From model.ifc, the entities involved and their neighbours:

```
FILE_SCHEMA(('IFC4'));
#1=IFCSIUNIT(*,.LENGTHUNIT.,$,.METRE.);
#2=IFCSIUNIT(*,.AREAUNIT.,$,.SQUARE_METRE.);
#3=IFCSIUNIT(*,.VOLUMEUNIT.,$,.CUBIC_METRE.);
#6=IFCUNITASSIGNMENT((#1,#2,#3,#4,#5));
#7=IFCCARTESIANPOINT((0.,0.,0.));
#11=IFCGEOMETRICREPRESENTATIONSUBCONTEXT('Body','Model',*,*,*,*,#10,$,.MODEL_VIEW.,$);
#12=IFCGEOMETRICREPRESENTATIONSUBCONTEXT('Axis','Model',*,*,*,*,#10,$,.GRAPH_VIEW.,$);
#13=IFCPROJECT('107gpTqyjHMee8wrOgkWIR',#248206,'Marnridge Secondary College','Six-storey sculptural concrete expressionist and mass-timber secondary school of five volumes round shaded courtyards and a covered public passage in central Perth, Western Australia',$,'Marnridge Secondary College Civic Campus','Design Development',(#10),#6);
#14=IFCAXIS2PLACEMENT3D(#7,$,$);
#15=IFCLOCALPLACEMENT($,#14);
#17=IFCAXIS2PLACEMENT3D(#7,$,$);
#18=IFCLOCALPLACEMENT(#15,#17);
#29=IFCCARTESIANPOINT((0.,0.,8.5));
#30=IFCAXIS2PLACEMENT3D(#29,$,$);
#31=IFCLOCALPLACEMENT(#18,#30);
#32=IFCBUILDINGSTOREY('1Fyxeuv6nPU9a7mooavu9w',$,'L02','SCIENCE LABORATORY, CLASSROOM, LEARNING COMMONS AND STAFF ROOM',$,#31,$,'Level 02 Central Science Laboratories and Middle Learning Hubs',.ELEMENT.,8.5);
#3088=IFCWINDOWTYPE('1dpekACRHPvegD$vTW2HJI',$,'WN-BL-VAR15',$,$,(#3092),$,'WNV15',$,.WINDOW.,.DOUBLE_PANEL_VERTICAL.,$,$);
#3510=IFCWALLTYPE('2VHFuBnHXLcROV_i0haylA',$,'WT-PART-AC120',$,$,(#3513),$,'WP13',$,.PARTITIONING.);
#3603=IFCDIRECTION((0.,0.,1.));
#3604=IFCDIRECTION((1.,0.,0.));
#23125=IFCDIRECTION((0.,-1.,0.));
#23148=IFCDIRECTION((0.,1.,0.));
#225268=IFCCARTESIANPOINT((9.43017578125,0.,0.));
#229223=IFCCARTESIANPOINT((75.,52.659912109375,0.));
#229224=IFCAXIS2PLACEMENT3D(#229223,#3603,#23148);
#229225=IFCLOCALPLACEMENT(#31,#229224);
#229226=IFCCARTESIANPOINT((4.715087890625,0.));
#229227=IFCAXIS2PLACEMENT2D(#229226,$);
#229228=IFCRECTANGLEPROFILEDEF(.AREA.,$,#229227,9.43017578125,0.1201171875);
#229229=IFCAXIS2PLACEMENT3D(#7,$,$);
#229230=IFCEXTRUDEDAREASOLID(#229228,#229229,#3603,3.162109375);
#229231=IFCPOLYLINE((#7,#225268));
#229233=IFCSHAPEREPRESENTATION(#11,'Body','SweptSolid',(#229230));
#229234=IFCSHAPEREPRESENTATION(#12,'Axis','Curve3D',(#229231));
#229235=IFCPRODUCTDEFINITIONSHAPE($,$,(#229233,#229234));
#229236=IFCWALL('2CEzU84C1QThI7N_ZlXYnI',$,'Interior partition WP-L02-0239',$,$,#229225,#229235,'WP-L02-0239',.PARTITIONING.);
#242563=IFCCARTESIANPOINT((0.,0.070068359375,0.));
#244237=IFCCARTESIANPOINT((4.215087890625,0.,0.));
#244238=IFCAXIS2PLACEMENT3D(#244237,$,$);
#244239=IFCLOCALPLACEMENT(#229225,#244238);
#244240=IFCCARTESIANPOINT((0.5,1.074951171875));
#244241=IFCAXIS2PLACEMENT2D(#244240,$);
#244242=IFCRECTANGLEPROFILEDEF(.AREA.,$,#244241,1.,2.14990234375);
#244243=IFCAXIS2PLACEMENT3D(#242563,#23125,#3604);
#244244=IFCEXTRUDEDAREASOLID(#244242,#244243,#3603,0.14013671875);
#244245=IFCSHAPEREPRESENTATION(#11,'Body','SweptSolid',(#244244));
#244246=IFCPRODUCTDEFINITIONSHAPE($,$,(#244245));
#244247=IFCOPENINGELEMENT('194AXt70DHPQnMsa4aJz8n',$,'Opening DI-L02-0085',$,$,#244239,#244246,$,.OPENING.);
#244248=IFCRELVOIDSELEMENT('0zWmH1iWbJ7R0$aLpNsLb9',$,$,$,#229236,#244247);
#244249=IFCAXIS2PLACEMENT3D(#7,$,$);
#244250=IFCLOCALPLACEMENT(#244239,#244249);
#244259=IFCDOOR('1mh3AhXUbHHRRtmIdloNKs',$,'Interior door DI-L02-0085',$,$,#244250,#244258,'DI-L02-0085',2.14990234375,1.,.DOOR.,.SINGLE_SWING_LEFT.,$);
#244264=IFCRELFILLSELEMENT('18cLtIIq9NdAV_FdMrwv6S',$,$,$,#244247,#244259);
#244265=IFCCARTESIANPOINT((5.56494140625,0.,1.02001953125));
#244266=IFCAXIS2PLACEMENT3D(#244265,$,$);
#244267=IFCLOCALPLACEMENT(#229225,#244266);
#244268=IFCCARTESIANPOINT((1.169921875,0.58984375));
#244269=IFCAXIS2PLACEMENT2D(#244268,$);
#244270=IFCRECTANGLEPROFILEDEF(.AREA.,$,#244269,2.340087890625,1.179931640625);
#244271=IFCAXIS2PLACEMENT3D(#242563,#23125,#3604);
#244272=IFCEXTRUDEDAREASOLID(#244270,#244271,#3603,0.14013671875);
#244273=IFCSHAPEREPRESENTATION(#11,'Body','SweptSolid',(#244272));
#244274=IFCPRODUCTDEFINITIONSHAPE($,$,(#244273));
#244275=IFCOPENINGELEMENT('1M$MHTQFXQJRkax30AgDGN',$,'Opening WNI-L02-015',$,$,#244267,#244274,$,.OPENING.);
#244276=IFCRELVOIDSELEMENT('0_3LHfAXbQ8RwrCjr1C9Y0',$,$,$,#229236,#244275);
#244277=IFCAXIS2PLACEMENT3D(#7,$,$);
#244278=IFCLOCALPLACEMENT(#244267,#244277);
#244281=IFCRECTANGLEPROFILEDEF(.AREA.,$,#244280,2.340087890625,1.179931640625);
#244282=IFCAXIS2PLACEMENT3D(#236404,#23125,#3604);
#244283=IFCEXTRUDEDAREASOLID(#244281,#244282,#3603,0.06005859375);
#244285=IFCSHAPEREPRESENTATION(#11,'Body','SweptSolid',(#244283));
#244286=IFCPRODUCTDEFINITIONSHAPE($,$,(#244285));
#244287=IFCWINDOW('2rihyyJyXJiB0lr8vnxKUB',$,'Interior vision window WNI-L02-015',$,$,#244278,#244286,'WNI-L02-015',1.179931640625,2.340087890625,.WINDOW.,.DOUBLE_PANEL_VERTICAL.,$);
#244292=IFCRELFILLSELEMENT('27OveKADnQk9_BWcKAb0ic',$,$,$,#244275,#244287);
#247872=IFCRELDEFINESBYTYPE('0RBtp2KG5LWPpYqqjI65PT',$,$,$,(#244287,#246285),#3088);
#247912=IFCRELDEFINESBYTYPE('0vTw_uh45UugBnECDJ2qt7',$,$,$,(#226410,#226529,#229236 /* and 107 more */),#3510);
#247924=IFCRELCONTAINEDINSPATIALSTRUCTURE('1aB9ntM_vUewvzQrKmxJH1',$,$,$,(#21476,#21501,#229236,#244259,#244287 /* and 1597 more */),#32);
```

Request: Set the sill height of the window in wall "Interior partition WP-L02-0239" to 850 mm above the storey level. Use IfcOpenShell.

```python
import numpy as np
import ifcopenshell
import ifcopenshell.api.geometry
import ifcopenshell.geom
import ifcopenshell.util.element
import ifcopenshell.util.placement
import ifcopenshell.util.shape
import ifcopenshell.util.unit

model = ifcopenshell.open("model.ifc")
unit_scale = ifcopenshell.util.unit.calculate_unit_scale(model)

window = model.by_guid("2rihyyJyXJiB0lr8vnxKUB")
opening = window.FillsVoids[0].RelatingOpeningElement
storey = ifcopenshell.util.element.get_container(window, ifc_class="IfcBuildingStorey")
level = ifcopenshell.util.placement.get_local_placement(storey.ObjectPlacement)[2, 3]

# The opening's origin need not be at the sill, so measure its lowest point.
shape = ifcopenshell.geom.create_shape(ifcopenshell.geom.settings(), opening)
bottom = ifcopenshell.util.shape.get_shape_bottom_elevation(shape, shape.geometry) / unit_scale
dz = level + 0.85 / unit_scale - bottom

shift = np.array([0.0, 0.0, dz])
# The window is placed relative to its opening, so it follows when the opening moves.
matrix = ifcopenshell.util.placement.get_local_placement(opening.ObjectPlacement)
matrix[:3, 3] += shift
ifcopenshell.api.geometry.edit_object_placement(
    model, product=opening, matrix=matrix, is_si=False, should_transform_children=True
)

print(f"moved by {dz * unit_scale:+.3f} m")

model.write("model_rev.ifc")
```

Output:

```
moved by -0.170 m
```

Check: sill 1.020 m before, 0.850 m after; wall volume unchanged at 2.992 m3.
